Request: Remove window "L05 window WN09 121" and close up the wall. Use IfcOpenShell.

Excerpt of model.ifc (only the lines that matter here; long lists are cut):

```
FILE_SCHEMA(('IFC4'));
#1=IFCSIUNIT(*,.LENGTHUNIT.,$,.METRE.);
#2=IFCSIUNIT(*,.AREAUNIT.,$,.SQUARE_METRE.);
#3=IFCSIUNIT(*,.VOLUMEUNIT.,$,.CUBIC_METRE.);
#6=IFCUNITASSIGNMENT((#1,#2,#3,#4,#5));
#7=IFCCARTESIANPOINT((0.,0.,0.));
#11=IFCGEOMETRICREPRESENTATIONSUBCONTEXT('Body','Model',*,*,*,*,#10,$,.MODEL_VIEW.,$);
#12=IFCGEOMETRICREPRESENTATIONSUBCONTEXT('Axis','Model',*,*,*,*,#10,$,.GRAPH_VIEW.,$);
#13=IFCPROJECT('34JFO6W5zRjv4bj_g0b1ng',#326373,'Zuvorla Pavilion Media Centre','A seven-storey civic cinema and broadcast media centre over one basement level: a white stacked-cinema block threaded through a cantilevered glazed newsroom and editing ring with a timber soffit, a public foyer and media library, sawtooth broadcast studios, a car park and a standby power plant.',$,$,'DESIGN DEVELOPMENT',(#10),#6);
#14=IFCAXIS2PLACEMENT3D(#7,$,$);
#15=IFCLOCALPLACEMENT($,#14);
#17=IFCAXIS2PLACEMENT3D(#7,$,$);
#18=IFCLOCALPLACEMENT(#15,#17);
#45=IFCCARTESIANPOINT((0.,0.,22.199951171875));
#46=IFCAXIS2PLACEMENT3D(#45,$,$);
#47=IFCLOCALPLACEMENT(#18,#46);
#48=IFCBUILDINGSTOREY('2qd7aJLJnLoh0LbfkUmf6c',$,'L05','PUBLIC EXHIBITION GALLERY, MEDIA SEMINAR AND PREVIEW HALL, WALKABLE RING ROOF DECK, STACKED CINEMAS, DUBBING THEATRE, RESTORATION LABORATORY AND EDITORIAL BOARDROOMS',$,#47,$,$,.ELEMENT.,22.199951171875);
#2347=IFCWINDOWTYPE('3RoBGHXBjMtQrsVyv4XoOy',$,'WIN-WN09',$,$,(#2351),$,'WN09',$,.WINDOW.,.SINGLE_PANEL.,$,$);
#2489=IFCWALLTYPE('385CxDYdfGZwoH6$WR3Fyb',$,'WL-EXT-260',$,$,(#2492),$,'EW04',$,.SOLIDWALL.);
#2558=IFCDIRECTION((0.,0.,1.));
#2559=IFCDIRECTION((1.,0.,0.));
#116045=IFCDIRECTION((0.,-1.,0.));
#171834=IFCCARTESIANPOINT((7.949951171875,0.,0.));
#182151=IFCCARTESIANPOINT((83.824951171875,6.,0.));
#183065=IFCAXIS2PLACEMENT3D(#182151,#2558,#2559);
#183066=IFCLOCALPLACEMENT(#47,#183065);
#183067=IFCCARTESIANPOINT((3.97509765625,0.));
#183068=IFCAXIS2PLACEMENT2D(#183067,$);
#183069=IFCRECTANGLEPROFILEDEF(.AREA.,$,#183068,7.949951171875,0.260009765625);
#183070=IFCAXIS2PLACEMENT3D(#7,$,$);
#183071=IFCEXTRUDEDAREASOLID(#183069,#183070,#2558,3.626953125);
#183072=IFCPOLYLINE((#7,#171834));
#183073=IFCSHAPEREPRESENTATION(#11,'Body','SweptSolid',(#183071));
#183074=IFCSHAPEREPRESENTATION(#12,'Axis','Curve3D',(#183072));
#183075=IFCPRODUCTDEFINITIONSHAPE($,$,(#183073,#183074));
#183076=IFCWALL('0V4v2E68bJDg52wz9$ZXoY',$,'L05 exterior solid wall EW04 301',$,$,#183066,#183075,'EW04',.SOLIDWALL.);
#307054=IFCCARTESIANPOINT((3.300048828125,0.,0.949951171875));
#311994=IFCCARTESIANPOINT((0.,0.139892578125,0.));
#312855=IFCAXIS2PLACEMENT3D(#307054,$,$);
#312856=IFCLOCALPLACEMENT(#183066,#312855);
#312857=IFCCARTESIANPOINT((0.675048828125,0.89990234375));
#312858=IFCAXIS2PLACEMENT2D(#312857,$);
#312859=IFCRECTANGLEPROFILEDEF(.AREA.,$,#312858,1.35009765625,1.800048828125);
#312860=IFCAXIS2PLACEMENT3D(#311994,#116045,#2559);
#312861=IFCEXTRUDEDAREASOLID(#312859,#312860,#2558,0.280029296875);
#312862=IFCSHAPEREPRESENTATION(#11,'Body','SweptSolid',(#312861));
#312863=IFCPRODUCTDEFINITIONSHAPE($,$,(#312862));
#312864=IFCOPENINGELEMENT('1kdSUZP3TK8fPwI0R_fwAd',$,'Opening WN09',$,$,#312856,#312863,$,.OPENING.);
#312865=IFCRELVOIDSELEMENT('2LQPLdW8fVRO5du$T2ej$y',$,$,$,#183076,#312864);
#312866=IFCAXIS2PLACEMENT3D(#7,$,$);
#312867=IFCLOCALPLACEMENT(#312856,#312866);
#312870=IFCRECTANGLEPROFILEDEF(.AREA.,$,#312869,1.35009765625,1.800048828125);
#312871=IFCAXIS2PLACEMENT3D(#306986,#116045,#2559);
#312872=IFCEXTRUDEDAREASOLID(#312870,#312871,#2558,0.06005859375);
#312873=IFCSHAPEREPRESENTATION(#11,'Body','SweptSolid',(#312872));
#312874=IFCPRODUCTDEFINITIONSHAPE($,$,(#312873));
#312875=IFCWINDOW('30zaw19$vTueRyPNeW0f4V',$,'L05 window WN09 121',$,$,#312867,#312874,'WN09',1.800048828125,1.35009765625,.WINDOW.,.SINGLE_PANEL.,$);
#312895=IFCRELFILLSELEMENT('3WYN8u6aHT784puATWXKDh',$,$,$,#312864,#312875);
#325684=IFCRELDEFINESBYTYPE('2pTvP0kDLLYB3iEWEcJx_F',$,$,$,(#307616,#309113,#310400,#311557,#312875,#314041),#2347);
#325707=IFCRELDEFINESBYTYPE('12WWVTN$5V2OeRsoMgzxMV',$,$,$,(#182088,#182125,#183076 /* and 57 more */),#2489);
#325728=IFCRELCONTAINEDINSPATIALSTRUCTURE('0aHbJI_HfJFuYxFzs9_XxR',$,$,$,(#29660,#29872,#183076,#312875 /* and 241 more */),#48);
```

```python
import ifcopenshell
import ifcopenshell.api.feature
import ifcopenshell.api.root
import ifcopenshell.geom
import ifcopenshell.util.shape

model = ifcopenshell.open("model.ifc")
settings = ifcopenshell.geom.settings()


def volume(element):
    """Net volume in cubic metres, openings subtracted."""
    shape = ifcopenshell.geom.create_shape(settings, element)
    return ifcopenshell.util.shape.get_volume(shape.geometry)


window = model.by_guid("30zaw19$vTueRyPNeW0f4V")
opening = window.FillsVoids[0].RelatingOpeningElement
wall = opening.VoidsElements[0].RelatingBuildingElement
before = volume(wall)

ifcopenshell.api.root.remove_product(model, product=window)
ifcopenshell.api.feature.remove_feature(model, feature=opening)

after = volume(wall)

print(f"wall volume {before:.3f} -> {after:.3f} m3")

model.write("model_updated.ifc")
```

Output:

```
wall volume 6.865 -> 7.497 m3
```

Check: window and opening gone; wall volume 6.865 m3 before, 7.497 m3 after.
